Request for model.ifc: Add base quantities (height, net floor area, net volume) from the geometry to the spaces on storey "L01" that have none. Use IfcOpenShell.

First a look at what the model holds.

```python
import ifcopenshell
import ifcopenshell.util.element
import ifcopenshell.util.unit

model = ifcopenshell.open("model.ifc")
print(model.schema)
for unit_type in ("LENGTHUNIT", "AREAUNIT", "VOLUMEUNIT"):
    print(unit_type, ifcopenshell.util.unit.calculate_unit_scale(model, unit_type))
storey = next(s for s in model.by_type("IfcBuildingStorey") if s.Name == "L01")
spaces = [e for e in ifcopenshell.util.element.get_decomposition(storey) if e.is_a("IfcSpace")]
for e in sorted(spaces, key=lambda e: e.id()):
    print(e.id(), e.is_a(), e.Name, list(ifcopenshell.util.element.get_psets(e, qtos_only=True)), sep=" | ")
```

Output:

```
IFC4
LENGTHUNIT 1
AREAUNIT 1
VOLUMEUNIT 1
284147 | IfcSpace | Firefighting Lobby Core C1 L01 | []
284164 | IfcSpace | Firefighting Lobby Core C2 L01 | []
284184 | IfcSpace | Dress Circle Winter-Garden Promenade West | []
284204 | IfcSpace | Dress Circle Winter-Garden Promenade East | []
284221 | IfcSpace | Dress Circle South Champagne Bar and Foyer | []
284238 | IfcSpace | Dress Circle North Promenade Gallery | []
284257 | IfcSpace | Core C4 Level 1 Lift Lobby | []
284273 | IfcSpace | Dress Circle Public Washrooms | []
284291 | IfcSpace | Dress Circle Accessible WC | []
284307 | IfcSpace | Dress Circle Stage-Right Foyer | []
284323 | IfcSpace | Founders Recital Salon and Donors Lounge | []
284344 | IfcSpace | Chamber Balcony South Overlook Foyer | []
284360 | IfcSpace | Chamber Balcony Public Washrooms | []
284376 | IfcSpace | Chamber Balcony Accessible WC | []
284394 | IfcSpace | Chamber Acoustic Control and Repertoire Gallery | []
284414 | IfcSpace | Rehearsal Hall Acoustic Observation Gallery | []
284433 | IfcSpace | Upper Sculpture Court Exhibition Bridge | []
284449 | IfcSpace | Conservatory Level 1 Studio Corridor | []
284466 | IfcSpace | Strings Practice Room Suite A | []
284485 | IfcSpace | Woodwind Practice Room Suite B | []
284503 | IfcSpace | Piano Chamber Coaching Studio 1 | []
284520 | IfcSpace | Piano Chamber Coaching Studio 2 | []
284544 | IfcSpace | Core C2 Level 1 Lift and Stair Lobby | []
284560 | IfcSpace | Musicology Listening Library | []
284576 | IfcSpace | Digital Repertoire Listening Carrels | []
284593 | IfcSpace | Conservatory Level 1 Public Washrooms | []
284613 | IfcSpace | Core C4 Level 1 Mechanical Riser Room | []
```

```python
import ifcopenshell
import ifcopenshell.api.pset
import ifcopenshell.geom
import ifcopenshell.util.element
import ifcopenshell.util.shape
import ifcopenshell.util.unit

model = ifcopenshell.open("model.ifc")
unit_scale = ifcopenshell.util.unit.calculate_unit_scale(model)
area_scale = ifcopenshell.util.unit.calculate_unit_scale(model, "AREAUNIT")
volume_scale = ifcopenshell.util.unit.calculate_unit_scale(model, "VOLUMEUNIT")
settings = ifcopenshell.geom.settings()

storey = next(s for s in model.by_type("IfcBuildingStorey") if s.Name == "L01")
spaces = [e for e in ifcopenshell.util.element.get_decomposition(storey) if e.is_a("IfcSpace")]

for e in sorted(spaces, key=lambda e: e.id()):
    if ifcopenshell.util.element.get_psets(e, qtos_only=True, should_inherit=False):
        continue
    # Geometry comes back in metres, in the element's own axes.
    shape = ifcopenshell.geom.create_shape(settings, e)
    values = {
        "Height": ifcopenshell.util.shape.get_z(shape.geometry) / unit_scale,
        "NetFloorArea": ifcopenshell.util.shape.get_footprint_area(shape.geometry) / area_scale,
        "NetVolume": ifcopenshell.util.shape.get_volume(shape.geometry) / volume_scale,
    }
    qto = ifcopenshell.api.pset.add_qto(model, product=e, name="Qto_SpaceBaseQuantities")
    ifcopenshell.api.pset.edit_qto(model, qto=qto, properties=values)
    print(e.id(), {k: round(v, 3) for k, v in values.items()})

model.write("model_updated.ifc")
```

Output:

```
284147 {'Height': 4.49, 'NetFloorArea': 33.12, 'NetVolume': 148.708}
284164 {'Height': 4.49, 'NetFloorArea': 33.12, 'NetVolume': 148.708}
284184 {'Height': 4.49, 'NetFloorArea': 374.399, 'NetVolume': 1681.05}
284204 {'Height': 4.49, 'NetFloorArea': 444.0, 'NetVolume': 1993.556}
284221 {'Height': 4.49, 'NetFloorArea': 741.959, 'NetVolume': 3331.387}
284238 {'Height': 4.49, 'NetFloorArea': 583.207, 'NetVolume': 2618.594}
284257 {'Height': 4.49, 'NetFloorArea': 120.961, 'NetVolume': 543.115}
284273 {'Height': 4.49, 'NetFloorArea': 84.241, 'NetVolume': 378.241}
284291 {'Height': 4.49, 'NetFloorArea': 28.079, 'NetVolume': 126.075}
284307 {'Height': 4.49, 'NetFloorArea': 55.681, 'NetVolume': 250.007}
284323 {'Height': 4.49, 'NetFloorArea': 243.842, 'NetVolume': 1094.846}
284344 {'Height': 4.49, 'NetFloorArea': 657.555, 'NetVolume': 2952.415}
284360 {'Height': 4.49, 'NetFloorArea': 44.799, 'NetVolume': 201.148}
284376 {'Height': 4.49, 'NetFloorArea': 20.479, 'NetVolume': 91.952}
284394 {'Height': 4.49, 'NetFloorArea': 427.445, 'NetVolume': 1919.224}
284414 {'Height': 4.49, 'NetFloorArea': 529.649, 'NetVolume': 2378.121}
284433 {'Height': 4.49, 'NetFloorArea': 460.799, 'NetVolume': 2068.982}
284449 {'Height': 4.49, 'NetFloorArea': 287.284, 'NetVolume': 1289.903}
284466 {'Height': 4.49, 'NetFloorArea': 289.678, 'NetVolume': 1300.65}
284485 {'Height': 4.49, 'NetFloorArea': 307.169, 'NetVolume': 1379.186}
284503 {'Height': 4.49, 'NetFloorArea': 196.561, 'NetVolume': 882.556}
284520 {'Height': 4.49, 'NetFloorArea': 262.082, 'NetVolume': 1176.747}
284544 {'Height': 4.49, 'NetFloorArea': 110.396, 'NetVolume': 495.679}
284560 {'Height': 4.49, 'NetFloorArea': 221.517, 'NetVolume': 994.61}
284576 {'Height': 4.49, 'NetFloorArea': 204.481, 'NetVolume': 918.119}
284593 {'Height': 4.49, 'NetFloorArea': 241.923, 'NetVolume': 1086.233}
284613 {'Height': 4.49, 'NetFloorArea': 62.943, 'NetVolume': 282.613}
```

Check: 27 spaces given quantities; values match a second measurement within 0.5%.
